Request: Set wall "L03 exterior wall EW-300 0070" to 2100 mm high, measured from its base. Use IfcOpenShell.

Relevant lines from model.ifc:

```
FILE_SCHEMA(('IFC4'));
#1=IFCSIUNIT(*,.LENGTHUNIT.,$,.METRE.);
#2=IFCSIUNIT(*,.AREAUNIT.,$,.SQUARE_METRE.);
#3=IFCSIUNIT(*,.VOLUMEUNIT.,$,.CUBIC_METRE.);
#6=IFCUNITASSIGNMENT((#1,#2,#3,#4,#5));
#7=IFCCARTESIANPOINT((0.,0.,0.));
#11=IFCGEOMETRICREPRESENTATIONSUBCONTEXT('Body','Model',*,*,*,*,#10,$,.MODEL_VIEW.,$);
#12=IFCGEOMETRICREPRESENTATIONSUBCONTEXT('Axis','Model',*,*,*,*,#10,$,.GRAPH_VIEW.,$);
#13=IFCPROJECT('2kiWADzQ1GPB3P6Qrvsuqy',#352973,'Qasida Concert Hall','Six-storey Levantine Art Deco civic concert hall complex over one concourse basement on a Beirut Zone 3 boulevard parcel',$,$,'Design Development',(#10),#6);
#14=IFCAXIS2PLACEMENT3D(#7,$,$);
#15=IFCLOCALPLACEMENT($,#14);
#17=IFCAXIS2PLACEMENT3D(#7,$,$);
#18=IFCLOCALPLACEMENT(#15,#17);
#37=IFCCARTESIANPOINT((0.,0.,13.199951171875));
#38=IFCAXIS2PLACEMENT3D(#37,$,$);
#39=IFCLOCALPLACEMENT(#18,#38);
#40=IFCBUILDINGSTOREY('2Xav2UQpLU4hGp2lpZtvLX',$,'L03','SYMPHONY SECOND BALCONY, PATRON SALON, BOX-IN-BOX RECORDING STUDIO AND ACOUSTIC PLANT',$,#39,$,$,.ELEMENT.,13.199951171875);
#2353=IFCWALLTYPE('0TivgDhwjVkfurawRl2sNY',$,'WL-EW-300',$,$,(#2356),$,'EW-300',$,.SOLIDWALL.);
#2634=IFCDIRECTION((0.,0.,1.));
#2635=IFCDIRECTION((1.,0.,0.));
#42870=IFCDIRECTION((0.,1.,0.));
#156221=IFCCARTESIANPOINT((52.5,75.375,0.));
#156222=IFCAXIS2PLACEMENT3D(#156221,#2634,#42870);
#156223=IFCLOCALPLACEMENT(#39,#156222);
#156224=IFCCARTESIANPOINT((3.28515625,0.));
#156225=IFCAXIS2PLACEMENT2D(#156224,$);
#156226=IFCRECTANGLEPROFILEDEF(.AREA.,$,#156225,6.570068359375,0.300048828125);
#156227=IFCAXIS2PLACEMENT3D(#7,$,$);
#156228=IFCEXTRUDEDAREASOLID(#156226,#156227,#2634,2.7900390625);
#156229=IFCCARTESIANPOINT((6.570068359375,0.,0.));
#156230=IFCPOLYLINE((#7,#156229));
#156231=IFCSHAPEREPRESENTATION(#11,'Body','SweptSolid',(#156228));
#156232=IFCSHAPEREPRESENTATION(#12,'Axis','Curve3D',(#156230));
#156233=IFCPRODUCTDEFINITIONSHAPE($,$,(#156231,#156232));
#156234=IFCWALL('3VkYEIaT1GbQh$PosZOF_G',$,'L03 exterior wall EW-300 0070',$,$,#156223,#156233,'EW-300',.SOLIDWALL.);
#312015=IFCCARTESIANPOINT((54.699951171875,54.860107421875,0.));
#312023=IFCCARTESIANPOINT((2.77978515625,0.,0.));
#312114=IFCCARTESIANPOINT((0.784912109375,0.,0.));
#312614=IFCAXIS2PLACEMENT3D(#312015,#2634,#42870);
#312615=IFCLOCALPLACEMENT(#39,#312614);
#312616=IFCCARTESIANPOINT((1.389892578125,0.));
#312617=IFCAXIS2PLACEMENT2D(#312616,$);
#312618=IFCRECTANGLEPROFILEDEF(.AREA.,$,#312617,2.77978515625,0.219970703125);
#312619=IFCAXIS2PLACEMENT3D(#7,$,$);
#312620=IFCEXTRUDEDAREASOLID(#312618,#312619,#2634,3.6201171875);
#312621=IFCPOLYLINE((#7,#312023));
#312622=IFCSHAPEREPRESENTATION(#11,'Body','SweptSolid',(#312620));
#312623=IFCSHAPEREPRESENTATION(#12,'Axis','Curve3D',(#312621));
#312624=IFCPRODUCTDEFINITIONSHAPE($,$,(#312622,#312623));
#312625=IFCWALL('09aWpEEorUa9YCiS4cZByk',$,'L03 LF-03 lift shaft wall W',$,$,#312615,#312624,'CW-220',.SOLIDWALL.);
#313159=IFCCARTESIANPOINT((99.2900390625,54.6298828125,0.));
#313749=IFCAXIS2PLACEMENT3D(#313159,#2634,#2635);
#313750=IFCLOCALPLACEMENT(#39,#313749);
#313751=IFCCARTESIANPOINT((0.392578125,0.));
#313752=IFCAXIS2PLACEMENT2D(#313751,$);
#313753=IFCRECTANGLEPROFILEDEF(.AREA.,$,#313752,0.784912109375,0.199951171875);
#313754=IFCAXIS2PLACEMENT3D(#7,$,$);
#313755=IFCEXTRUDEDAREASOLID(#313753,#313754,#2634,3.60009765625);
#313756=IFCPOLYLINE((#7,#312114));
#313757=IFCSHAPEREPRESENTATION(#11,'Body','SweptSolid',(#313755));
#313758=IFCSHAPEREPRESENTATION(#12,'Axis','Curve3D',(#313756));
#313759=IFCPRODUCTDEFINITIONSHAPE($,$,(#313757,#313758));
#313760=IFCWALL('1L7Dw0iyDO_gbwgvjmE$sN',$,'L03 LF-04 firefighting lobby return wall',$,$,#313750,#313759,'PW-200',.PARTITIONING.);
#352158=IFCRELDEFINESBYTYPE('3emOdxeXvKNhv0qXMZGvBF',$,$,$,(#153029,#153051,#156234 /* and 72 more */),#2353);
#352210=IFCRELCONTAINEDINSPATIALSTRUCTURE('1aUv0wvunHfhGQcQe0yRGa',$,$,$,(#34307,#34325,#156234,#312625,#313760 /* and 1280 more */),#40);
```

```python
import ifcopenshell
import ifcopenshell.geom
import ifcopenshell.util.representation
import ifcopenshell.util.shape

model = ifcopenshell.open("model.ifc")
settings = ifcopenshell.geom.settings()


def volume(element):
    """Net volume in cubic metres, openings subtracted."""
    shape = ifcopenshell.geom.create_shape(settings, element)
    return ifcopenshell.util.shape.get_volume(shape.geometry)


wall = model.by_id(156234)
before = volume(wall)

body = ifcopenshell.util.representation.get_representation(wall, "Model", "Body")
solid = body.Items[0]
old_height = solid.Depth
solid.Depth = 2.1
after = volume(wall)

print(f"height {old_height:g} -> {solid.Depth:g}, volume {before:.3f} -> {after:.3f} m3")

model.write("model_rev.ifc")
```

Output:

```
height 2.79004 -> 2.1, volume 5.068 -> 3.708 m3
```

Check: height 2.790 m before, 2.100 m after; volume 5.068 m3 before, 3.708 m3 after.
